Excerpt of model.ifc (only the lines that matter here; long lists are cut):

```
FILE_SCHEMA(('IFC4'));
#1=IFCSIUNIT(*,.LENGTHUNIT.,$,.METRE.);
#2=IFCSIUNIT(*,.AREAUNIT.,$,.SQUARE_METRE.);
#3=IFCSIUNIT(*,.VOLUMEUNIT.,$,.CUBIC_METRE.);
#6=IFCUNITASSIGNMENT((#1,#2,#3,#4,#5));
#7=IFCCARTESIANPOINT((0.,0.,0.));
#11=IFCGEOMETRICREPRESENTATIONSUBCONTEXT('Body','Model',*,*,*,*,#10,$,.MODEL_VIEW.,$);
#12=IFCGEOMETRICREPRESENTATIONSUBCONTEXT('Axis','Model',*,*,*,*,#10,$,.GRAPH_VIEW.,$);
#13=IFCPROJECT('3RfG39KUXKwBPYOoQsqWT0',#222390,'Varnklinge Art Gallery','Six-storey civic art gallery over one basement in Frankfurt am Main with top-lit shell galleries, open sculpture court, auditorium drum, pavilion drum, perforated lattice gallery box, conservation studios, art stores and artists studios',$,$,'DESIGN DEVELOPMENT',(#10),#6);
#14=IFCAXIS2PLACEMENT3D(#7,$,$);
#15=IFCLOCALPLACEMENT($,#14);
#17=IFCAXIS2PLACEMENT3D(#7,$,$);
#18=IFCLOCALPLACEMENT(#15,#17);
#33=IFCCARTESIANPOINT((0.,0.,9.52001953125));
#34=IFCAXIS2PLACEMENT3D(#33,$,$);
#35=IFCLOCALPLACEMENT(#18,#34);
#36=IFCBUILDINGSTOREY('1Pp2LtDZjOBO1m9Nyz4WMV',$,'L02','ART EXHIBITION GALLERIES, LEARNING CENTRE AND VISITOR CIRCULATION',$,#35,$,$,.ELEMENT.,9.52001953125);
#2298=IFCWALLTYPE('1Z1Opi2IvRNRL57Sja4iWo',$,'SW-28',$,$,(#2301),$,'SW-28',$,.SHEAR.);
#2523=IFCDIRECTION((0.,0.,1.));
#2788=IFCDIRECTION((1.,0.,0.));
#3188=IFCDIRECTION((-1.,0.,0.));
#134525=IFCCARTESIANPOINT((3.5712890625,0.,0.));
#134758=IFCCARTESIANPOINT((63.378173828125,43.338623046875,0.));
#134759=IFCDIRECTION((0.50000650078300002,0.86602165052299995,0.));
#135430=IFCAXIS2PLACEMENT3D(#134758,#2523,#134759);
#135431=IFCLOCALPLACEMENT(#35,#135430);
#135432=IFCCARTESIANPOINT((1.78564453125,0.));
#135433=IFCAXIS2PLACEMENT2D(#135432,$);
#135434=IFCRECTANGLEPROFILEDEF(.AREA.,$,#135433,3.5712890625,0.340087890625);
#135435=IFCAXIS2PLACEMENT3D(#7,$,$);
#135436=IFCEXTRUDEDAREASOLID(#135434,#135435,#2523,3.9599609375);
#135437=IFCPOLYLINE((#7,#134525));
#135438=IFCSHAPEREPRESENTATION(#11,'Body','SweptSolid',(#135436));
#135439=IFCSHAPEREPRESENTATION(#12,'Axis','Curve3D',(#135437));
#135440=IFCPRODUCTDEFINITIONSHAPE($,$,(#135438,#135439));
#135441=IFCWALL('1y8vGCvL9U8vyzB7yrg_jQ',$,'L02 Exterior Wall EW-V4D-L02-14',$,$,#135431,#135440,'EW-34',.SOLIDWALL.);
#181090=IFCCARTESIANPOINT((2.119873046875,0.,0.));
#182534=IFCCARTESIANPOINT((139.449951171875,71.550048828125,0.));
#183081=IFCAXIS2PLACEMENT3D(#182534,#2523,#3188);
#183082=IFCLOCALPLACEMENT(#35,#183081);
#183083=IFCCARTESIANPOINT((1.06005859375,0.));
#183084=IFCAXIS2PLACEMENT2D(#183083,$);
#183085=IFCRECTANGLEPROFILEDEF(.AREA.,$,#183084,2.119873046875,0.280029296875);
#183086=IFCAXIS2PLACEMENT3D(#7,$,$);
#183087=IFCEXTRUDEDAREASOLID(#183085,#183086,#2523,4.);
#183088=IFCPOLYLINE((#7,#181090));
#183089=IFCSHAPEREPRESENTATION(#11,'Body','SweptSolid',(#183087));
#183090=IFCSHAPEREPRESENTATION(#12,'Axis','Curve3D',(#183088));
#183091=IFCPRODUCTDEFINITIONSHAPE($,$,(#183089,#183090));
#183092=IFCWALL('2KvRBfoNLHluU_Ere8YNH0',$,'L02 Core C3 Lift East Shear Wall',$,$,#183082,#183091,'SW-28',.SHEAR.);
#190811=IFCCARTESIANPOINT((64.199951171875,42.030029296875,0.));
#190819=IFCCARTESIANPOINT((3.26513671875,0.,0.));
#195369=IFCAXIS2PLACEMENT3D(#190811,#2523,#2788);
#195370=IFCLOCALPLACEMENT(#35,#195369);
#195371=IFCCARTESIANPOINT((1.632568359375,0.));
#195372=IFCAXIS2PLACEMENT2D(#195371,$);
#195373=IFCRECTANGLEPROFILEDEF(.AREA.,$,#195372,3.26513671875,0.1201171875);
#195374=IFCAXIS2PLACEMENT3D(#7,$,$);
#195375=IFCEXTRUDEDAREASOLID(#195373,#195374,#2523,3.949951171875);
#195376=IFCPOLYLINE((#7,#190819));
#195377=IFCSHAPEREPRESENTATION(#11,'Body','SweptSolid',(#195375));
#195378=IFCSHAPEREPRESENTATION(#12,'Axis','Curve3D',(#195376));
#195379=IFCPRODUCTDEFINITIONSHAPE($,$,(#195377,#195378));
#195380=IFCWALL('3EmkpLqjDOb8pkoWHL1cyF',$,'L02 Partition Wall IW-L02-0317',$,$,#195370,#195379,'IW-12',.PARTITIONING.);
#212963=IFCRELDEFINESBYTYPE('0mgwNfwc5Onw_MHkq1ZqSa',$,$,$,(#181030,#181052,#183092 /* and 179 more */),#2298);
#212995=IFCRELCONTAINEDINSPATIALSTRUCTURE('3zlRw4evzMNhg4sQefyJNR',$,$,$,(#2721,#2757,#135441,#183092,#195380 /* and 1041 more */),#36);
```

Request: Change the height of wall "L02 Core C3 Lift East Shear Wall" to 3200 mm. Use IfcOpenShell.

```python
import ifcopenshell
import ifcopenshell.geom
import ifcopenshell.util.representation
import ifcopenshell.util.shape
import ifcopenshell.util.unit

model = ifcopenshell.open("model.ifc")
unit_scale = ifcopenshell.util.unit.calculate_unit_scale(model)
settings = ifcopenshell.geom.settings()


def volume(element):
    """Net volume in cubic metres, openings subtracted."""
    shape = ifcopenshell.geom.create_shape(settings, element)
    return ifcopenshell.util.shape.get_volume(shape.geometry)


wall = model.by_id(183092)
before = volume(wall)

body = ifcopenshell.util.representation.get_representation(wall, "Model", "Body")
solid = body.Items[0]
old_height = solid.Depth
solid.Depth = 3.2 / unit_scale
after = volume(wall)

print(f"height {old_height:g} -> {solid.Depth:g}, volume {before:.3f} -> {after:.3f} m3")

model.write("model-out.ifc")
```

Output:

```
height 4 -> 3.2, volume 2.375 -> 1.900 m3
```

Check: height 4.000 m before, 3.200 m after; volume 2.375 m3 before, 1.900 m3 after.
